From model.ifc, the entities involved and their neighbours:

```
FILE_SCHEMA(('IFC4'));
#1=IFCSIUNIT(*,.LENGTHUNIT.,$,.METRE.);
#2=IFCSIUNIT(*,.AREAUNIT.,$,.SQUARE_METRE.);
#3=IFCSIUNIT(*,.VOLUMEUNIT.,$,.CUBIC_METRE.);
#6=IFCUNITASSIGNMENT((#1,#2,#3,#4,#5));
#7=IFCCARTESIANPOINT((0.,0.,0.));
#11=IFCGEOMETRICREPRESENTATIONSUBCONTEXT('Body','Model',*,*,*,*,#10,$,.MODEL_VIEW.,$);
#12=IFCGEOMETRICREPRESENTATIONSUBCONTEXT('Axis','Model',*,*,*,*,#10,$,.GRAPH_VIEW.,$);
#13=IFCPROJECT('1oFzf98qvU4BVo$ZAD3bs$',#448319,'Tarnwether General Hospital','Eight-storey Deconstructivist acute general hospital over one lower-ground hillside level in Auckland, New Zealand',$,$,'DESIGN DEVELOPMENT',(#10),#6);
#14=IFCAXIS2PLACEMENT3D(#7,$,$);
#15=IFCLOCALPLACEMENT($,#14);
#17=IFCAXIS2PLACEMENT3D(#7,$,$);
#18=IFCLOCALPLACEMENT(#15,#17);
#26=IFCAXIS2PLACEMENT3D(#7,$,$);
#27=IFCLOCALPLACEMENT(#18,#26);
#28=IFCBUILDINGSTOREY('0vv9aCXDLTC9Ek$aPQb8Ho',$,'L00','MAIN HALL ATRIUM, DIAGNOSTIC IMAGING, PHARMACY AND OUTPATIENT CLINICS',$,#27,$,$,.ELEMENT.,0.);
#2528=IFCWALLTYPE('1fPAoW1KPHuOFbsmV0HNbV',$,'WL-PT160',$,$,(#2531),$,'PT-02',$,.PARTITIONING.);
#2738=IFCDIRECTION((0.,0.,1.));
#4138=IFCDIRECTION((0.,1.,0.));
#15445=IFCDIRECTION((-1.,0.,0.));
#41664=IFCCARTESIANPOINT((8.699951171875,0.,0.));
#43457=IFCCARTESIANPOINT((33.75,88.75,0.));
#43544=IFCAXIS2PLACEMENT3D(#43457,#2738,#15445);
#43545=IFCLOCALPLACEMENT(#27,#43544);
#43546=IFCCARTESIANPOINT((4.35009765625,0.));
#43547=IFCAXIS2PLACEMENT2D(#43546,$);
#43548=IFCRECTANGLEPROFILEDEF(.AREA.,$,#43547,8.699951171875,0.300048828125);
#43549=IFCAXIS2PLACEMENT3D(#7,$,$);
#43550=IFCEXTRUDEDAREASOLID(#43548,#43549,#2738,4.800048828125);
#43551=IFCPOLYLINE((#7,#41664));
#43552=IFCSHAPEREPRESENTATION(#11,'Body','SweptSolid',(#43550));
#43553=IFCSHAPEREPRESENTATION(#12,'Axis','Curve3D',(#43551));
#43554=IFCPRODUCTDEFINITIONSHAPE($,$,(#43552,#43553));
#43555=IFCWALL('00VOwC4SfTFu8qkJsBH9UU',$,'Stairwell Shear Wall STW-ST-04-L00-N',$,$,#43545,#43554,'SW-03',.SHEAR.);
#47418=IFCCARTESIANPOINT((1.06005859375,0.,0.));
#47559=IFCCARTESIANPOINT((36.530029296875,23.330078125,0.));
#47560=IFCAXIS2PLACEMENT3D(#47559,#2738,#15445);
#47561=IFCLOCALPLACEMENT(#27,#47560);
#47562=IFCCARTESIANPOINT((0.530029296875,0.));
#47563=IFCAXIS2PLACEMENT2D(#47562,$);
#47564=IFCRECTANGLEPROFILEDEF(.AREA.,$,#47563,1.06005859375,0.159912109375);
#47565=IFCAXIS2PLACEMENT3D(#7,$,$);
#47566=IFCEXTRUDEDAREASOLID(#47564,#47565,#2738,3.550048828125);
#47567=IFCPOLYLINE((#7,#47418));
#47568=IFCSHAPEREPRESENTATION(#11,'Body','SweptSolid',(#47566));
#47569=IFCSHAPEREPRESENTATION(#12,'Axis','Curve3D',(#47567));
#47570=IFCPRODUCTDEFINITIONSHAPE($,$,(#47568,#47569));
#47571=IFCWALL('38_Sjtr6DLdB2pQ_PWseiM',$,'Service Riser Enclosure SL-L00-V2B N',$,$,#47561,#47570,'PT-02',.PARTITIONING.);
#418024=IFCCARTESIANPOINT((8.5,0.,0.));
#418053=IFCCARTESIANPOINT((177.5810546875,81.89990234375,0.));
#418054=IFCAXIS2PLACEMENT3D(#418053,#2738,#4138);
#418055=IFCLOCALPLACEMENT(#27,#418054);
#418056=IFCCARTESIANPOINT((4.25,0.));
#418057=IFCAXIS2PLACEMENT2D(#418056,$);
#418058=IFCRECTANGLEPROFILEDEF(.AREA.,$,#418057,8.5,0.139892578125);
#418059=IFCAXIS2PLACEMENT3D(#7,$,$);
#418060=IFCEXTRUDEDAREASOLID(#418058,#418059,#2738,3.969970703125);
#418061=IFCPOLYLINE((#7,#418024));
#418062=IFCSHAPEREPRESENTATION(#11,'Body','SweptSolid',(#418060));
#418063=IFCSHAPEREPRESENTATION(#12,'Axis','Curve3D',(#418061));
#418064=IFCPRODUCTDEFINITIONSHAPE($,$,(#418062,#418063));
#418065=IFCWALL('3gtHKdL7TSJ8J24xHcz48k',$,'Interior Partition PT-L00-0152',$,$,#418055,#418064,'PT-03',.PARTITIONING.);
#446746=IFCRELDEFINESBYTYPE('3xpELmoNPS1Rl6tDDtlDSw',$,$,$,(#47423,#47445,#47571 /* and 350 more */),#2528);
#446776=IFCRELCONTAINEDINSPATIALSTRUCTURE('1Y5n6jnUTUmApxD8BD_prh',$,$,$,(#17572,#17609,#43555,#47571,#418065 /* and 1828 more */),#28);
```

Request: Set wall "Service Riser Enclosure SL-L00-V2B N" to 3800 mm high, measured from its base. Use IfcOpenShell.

```python
import ifcopenshell
import ifcopenshell.geom
import ifcopenshell.util.representation
import ifcopenshell.util.shape
import ifcopenshell.util.unit

model = ifcopenshell.open("model.ifc")
unit_scale = ifcopenshell.util.unit.calculate_unit_scale(model)
settings = ifcopenshell.geom.settings()


def volume(element):
    """Net volume in cubic metres, openings subtracted."""
    shape = ifcopenshell.geom.create_shape(settings, element)
    return ifcopenshell.util.shape.get_volume(shape.geometry)


wall = model.by_guid("38_Sjtr6DLdB2pQ_PWseiM")
before = volume(wall)

body = ifcopenshell.util.representation.get_representation(wall, "Model", "Body")
solid = body.Items[0]
old_height = solid.Depth
solid.Depth = 3.8 / unit_scale
after = volume(wall)

print(f"height {old_height:g} -> {solid.Depth:g}, volume {before:.3f} -> {after:.3f} m3")

model.write("model_updated.ifc")
```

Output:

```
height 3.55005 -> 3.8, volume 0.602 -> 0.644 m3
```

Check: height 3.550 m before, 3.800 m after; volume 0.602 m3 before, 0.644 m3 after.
